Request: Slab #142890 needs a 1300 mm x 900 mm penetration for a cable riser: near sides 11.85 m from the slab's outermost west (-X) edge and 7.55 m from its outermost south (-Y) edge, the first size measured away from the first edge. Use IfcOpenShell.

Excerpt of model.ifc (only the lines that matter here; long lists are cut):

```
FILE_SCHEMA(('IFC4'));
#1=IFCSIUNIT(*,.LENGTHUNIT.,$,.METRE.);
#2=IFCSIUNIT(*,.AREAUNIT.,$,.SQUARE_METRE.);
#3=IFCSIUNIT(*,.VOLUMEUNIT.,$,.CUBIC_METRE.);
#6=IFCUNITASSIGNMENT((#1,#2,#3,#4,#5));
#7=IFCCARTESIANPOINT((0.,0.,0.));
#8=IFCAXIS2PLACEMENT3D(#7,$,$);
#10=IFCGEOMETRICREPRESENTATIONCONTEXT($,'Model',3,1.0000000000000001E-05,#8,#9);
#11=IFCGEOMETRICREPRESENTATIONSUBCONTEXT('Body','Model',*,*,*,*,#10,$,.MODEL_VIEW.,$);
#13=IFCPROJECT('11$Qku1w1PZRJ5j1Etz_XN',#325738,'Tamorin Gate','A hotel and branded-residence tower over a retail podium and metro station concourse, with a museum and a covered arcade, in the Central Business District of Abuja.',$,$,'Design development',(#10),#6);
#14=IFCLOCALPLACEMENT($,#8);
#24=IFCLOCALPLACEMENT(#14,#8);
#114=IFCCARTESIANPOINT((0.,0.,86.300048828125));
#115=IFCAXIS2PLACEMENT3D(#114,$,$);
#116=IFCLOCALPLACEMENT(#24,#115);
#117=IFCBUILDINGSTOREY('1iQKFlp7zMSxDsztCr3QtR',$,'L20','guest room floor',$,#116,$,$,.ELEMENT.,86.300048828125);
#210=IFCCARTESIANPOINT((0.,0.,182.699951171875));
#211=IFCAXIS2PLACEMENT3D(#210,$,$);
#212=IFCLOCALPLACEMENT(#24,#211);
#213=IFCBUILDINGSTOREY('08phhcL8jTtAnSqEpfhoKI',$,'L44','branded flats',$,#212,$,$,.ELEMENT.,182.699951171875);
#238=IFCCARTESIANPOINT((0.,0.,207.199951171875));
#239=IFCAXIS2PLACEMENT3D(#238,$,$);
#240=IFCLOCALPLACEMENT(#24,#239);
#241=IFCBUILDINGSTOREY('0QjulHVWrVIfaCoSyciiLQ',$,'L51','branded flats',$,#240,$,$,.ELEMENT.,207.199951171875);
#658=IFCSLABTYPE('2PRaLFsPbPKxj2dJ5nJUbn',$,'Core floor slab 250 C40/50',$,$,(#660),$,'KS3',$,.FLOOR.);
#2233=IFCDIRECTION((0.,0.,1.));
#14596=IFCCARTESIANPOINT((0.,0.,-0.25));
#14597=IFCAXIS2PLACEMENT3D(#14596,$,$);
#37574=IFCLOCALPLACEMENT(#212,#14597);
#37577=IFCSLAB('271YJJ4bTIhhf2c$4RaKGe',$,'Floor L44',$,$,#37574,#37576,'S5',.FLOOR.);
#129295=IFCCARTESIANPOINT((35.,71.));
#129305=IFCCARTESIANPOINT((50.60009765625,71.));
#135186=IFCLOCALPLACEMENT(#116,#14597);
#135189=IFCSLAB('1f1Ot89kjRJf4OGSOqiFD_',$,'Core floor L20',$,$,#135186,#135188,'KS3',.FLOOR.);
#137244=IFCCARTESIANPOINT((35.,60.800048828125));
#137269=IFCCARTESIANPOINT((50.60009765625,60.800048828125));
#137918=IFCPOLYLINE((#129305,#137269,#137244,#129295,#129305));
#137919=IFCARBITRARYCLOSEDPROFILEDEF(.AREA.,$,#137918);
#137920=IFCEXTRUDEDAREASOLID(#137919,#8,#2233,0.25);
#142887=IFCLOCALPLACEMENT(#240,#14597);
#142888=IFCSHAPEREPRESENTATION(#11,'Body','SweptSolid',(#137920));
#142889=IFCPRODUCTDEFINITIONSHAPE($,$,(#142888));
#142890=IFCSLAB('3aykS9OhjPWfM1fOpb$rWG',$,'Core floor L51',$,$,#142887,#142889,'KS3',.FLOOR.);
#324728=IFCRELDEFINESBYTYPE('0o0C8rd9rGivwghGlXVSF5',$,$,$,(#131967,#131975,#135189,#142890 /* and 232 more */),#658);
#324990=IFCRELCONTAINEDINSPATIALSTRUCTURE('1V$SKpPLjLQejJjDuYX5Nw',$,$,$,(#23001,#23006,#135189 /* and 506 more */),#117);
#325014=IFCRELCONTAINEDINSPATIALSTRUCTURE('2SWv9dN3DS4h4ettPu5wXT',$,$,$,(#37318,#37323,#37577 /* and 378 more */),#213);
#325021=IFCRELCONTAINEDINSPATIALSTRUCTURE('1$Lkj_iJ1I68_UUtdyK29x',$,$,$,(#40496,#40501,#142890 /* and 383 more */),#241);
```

```python
import numpy as np
import ifcopenshell
import ifcopenshell.api.feature
import ifcopenshell.api.geometry
import ifcopenshell.api.root
import ifcopenshell.geom
import ifcopenshell.util.placement
import ifcopenshell.util.representation
import ifcopenshell.util.shape
import ifcopenshell.util.unit

model = ifcopenshell.open("model.ifc")
unit_scale = ifcopenshell.util.unit.calculate_unit_scale(model)
settings = ifcopenshell.geom.settings()


def volume(element):
    """Net volume in cubic metres, openings subtracted."""
    shape = ifcopenshell.geom.create_shape(settings, element)
    return ifcopenshell.util.shape.get_volume(shape.geometry)


slab = model.by_guid("3aykS9OhjPWfM1fOpb$rWG")
before = volume(slab)

# Extent in the slab's own axes, in metres. The edges named are its -X and -Y sides.
slab_shape = ifcopenshell.geom.create_shape(settings, slab)
vertices = ifcopenshell.util.shape.get_vertices(slab_shape.geometry)
x_min, y_min, bottom = vertices.min(axis=0)
top = vertices[:, 2].max()

opening = ifcopenshell.api.root.create_entity(model, ifc_class="IfcOpeningElement", name="Cable riser opening", predefined_type="OPENING")
context = ifcopenshell.util.representation.get_context(model, "Model", "Body", "MODEL_VIEW")
width, depth = 1.3, 0.9
outline = [(0.0, 0.0), (width, 0.0), (width, depth), (0.0, depth), (0.0, 0.0)]
# Overshoot both faces by 50 mm so the cut is clean.
shape = ifcopenshell.api.geometry.add_slab_representation(
    model, context=context, depth=top - bottom + 0.1, polyline=outline
)
ifcopenshell.api.geometry.assign_representation(model, product=opening, representation=shape)

matrix = ifcopenshell.util.placement.get_local_placement(slab.ObjectPlacement)
matrix[:, 3] = matrix @ np.append(np.array([x_min + 11.85, y_min + 7.55, bottom - 0.05]) / unit_scale, 1.0)
ifcopenshell.api.geometry.edit_object_placement(model, product=opening, matrix=matrix, is_si=False)
ifcopenshell.api.feature.add_feature(model, feature=opening, element=slab)

after = volume(slab)

print(f"slab volume {before:.3f} -> {after:.3f} m3")

model.write("model_v2.ifc")
```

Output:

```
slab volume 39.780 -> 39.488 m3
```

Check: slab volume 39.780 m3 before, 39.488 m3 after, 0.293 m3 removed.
